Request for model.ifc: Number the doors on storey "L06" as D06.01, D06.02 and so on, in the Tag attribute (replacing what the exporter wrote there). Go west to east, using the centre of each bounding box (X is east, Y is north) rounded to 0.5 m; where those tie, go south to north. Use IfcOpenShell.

First a look at what the model holds.

```python
import ifcopenshell
import ifcopenshell.util.element
import ifcopenshell.util.placement

model = ifcopenshell.open("model.ifc")
print(model.schema)
storey = next(s for s in model.by_type("IfcBuildingStorey") if s.Name == "L06")
doors = [e for e in ifcopenshell.util.element.get_decomposition(storey) if e.is_a("IfcDoor")]
for e in sorted(doors, key=lambda e: e.id()):
    origin = ifcopenshell.util.placement.get_local_placement(e.ObjectPlacement)[:3, 3]
    print(e.id(), e.Tag, e.Name, origin.round(2) + 0.0, sep=" | ")
```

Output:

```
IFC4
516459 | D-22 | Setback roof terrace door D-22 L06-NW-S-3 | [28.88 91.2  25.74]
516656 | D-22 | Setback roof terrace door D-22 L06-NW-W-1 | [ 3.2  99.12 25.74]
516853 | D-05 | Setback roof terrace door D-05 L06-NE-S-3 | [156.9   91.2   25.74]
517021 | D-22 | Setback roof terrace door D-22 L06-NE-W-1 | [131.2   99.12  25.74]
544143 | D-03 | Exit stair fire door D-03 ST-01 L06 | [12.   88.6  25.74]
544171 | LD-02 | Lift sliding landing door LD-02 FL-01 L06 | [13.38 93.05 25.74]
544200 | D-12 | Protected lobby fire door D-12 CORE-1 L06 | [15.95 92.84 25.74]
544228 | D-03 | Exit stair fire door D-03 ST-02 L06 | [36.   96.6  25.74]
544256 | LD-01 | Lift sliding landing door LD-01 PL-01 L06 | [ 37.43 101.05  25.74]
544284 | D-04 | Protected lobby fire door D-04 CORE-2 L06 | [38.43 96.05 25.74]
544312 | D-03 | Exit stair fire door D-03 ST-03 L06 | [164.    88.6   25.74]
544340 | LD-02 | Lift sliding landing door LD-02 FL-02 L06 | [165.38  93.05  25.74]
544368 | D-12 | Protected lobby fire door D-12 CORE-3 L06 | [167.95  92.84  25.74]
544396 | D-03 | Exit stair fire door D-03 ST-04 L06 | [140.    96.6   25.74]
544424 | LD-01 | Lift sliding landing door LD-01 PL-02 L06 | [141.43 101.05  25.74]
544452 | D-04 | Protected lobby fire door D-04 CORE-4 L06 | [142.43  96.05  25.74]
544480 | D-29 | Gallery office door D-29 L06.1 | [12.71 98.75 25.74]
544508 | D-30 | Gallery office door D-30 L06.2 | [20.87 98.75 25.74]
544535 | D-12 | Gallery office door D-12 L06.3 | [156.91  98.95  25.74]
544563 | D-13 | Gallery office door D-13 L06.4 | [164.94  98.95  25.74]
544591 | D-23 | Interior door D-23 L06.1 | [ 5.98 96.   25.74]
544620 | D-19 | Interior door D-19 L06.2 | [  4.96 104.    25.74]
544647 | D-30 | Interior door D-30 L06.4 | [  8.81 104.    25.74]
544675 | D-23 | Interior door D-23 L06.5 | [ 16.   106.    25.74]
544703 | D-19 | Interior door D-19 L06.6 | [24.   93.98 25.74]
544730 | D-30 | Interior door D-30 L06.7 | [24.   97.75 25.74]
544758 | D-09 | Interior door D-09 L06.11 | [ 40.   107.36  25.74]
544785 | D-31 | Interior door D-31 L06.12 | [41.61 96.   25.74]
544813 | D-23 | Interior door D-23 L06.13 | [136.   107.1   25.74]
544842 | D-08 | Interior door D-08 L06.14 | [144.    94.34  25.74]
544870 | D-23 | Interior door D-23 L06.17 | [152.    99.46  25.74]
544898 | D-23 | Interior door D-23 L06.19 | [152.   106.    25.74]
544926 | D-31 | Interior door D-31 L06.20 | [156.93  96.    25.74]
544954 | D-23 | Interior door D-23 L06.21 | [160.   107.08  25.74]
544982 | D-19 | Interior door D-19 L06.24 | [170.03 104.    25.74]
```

```python
import ifcopenshell
import ifcopenshell.geom
import ifcopenshell.util.element
import ifcopenshell.util.shape

model = ifcopenshell.open("model.ifc")
settings = ifcopenshell.geom.settings()
settings.set("use-world-coords", True)


def centre(element):
    shape = ifcopenshell.geom.create_shape(settings, element)
    return ifcopenshell.util.shape.get_bbox_centroid(shape.geometry)


storey = next(s for s in model.by_type("IfcBuildingStorey") if s.Name == "L06")
doors = [e for e in ifcopenshell.util.element.get_decomposition(storey) if e.is_a("IfcDoor")]

# Insertion points can sit at a corner or the storey origin, so sort by the geometry (in metres).
centres = {e: centre(e) for e in doors}
doors.sort(key=lambda e: (round(centres[e][0] / 0.5), centres[e][1]))

for i, e in enumerate(doors, start=1):
    number = f"D06.{i:02d}"
    e.Tag = number
    print(e.id(), number)

model.write("model_v2.ifc")
```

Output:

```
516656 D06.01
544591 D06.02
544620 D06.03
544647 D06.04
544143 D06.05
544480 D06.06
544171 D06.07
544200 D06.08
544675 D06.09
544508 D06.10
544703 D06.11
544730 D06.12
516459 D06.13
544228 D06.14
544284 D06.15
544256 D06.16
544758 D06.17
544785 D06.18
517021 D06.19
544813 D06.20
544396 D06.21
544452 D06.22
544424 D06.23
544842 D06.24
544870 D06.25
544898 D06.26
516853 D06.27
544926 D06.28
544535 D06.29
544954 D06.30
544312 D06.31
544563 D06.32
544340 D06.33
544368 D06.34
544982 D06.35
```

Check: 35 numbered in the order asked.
